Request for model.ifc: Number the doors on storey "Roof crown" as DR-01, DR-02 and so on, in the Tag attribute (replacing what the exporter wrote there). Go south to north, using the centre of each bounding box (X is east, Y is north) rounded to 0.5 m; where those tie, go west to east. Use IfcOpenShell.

First a look at what the model holds.

```python
import ifcopenshell
import ifcopenshell.util.element
import ifcopenshell.util.placement

model = ifcopenshell.open("model.ifc")
print(model.schema)
storey = next(s for s in model.by_type("IfcBuildingStorey") if s.Name == "Roof crown")
doors = [e for e in ifcopenshell.util.element.get_decomposition(storey) if e.is_a("IfcDoor")]
for e in sorted(doors, key=lambda e: e.id()):
    origin = ifcopenshell.util.placement.get_local_placement(e.ObjectPlacement)[:3, 3]
    print(e.id(), e.Tag, e.Name, origin.round(2) + 0.0, sep=" | ")
```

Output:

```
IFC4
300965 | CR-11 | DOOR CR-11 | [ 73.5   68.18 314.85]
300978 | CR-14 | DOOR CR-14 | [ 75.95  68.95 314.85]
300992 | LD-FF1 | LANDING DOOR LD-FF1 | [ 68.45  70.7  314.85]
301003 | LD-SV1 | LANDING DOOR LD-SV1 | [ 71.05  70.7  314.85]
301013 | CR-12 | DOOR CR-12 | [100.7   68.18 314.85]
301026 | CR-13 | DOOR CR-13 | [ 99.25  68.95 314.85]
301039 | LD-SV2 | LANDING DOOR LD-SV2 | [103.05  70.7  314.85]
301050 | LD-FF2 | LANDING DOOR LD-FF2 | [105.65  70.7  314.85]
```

```python
import ifcopenshell
import ifcopenshell.geom
import ifcopenshell.util.element
import ifcopenshell.util.shape

model = ifcopenshell.open("model.ifc")
settings = ifcopenshell.geom.settings()
settings.set("use-world-coords", True)


def centre(element):
    shape = ifcopenshell.geom.create_shape(settings, element)
    return ifcopenshell.util.shape.get_bbox_centroid(shape.geometry)


storey = next(s for s in model.by_type("IfcBuildingStorey") if s.Name == "Roof crown")
doors = [e for e in ifcopenshell.util.element.get_decomposition(storey) if e.is_a("IfcDoor")]

# Insertion points can sit at a corner or the storey origin, so sort by the geometry (in metres).
centres = {e: centre(e) for e in doors}
doors.sort(key=lambda e: (round(centres[e][1] / 0.5), centres[e][0]))

for i, e in enumerate(doors, start=1):
    number = f"DR-{i:02d}"
    e.Tag = number
    print(e.id(), number)

model.write("model_v2.ifc")
```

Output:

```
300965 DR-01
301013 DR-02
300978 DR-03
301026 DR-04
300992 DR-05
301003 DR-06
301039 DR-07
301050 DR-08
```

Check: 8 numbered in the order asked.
